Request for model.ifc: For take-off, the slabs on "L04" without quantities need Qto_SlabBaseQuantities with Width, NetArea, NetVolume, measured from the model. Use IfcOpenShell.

First a look at what the model holds.

```python
import ifcopenshell
import ifcopenshell.util.element
import ifcopenshell.util.unit

model = ifcopenshell.open("model.ifc")
print(model.schema)
for unit_type in ("LENGTHUNIT", "AREAUNIT", "VOLUMEUNIT"):
    print(unit_type, ifcopenshell.util.unit.calculate_unit_scale(model, unit_type))
storey = next(s for s in model.by_type("IfcBuildingStorey") if s.Name == "L04")
slabs = [e for e in ifcopenshell.util.element.get_decomposition(storey) if e.is_a("IfcSlab")]
for e in sorted(slabs, key=lambda e: e.id()):
    print(e.id(), e.is_a(), e.Name, list(ifcopenshell.util.element.get_psets(e, qtos_only=True)), sep=" | ")
```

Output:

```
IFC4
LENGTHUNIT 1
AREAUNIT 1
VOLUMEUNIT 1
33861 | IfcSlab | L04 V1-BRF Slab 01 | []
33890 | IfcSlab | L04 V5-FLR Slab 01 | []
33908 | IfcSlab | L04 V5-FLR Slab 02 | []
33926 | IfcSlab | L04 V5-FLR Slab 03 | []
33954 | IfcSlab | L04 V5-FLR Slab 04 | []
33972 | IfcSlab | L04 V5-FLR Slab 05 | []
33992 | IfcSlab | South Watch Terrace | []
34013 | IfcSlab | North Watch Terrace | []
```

```python
import ifcopenshell
import ifcopenshell.api.pset
import ifcopenshell.geom
import ifcopenshell.util.element
import ifcopenshell.util.shape
import ifcopenshell.util.unit

model = ifcopenshell.open("model.ifc")
unit_scale = ifcopenshell.util.unit.calculate_unit_scale(model)
area_scale = ifcopenshell.util.unit.calculate_unit_scale(model, "AREAUNIT")
volume_scale = ifcopenshell.util.unit.calculate_unit_scale(model, "VOLUMEUNIT")
settings = ifcopenshell.geom.settings()

storey = next(s for s in model.by_type("IfcBuildingStorey") if s.Name == "L04")
slabs = [e for e in ifcopenshell.util.element.get_decomposition(storey) if e.is_a("IfcSlab")]

for e in sorted(slabs, key=lambda e: e.id()):
    if ifcopenshell.util.element.get_psets(e, qtos_only=True, should_inherit=False):
        continue
    # Geometry comes back in metres, in the element's own axes.
    shape = ifcopenshell.geom.create_shape(settings, e)
    values = {
        "Width": ifcopenshell.util.shape.get_z(shape.geometry) / unit_scale,
        "NetArea": ifcopenshell.util.shape.get_footprint_area(shape.geometry) / area_scale,
        "NetVolume": ifcopenshell.util.shape.get_volume(shape.geometry) / volume_scale,
    }
    qto = ifcopenshell.api.pset.add_qto(model, product=e, name="Qto_SlabBaseQuantities")
    ifcopenshell.api.pset.edit_qto(model, qto=qto, properties=values)
    print(e.id(), {k: round(v, 3) for k, v in values.items()})

model.write("model_edited.ifc")
```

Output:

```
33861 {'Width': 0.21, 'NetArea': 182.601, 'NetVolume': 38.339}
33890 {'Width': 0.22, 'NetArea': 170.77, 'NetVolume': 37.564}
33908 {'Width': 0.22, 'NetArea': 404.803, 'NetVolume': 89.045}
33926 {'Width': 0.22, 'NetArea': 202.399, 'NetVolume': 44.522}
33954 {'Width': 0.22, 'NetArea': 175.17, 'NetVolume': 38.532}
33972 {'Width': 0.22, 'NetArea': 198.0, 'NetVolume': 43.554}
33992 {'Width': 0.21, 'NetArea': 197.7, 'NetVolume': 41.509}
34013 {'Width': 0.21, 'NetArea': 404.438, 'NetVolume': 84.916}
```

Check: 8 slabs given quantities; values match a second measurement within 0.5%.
